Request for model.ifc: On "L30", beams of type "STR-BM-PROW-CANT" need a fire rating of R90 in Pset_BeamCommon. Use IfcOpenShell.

First a look at what the model holds.

```python
import ifcopenshell
import ifcopenshell.util.element

model = ifcopenshell.open("model.ifc")
print(model.schema)
storey = next(s for s in model.by_type("IfcBuildingStorey") if s.Name == "L30")
beams = [e for e in ifcopenshell.util.element.get_decomposition(storey) if e.is_a("IfcBeam")]
seen = {}
for e in beams:
    element_type = ifcopenshell.util.element.get_type(e)
    key = (element_type.Name if element_type != e and element_type else None, ifcopenshell.util.element.get_pset(e, "Pset_BeamCommon", "FireRating"))
    seen[key] = seen.get(key, 0) + 1
for (name, value), count in sorted(seen.items(), key=str):
    print(count, "x", name, "|", value)
```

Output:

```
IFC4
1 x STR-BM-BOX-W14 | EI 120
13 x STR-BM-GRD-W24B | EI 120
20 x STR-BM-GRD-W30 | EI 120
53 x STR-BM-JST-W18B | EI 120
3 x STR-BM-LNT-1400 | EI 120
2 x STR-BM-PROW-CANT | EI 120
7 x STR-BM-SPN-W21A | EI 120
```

```python
import ifcopenshell
import ifcopenshell.api.pset
import ifcopenshell.util.element

model = ifcopenshell.open("model.ifc")

storey = next(s for s in model.by_type("IfcBuildingStorey") if s.Name == "L30")
beams = [e for e in ifcopenshell.util.element.get_decomposition(storey) if e.is_a("IfcBeam")]

count = 0
for e in beams:
    element_type = ifcopenshell.util.element.get_type(e)
    if element_type in (None, e) or element_type.Name != "STR-BM-PROW-CANT":
        continue
    found = ifcopenshell.util.element.get_pset(e, "Pset_BeamCommon", should_inherit=False)
    if found:
        pset = model.by_id(found["id"])
        if len(ifcopenshell.util.element.get_elements_by_pset(pset)) > 1:
            pset = ifcopenshell.api.pset.unshare_pset(model, products=[e], pset=pset)[0]
    else:
        pset = ifcopenshell.api.pset.add_pset(model, product=e, name="Pset_BeamCommon")
    ifcopenshell.api.pset.edit_pset(model, pset=pset, properties={"FireRating": "R90"})
    count += 1

print(count, "beams updated")

model.write("model-out.ifc")
```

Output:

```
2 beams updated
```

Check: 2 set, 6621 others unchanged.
